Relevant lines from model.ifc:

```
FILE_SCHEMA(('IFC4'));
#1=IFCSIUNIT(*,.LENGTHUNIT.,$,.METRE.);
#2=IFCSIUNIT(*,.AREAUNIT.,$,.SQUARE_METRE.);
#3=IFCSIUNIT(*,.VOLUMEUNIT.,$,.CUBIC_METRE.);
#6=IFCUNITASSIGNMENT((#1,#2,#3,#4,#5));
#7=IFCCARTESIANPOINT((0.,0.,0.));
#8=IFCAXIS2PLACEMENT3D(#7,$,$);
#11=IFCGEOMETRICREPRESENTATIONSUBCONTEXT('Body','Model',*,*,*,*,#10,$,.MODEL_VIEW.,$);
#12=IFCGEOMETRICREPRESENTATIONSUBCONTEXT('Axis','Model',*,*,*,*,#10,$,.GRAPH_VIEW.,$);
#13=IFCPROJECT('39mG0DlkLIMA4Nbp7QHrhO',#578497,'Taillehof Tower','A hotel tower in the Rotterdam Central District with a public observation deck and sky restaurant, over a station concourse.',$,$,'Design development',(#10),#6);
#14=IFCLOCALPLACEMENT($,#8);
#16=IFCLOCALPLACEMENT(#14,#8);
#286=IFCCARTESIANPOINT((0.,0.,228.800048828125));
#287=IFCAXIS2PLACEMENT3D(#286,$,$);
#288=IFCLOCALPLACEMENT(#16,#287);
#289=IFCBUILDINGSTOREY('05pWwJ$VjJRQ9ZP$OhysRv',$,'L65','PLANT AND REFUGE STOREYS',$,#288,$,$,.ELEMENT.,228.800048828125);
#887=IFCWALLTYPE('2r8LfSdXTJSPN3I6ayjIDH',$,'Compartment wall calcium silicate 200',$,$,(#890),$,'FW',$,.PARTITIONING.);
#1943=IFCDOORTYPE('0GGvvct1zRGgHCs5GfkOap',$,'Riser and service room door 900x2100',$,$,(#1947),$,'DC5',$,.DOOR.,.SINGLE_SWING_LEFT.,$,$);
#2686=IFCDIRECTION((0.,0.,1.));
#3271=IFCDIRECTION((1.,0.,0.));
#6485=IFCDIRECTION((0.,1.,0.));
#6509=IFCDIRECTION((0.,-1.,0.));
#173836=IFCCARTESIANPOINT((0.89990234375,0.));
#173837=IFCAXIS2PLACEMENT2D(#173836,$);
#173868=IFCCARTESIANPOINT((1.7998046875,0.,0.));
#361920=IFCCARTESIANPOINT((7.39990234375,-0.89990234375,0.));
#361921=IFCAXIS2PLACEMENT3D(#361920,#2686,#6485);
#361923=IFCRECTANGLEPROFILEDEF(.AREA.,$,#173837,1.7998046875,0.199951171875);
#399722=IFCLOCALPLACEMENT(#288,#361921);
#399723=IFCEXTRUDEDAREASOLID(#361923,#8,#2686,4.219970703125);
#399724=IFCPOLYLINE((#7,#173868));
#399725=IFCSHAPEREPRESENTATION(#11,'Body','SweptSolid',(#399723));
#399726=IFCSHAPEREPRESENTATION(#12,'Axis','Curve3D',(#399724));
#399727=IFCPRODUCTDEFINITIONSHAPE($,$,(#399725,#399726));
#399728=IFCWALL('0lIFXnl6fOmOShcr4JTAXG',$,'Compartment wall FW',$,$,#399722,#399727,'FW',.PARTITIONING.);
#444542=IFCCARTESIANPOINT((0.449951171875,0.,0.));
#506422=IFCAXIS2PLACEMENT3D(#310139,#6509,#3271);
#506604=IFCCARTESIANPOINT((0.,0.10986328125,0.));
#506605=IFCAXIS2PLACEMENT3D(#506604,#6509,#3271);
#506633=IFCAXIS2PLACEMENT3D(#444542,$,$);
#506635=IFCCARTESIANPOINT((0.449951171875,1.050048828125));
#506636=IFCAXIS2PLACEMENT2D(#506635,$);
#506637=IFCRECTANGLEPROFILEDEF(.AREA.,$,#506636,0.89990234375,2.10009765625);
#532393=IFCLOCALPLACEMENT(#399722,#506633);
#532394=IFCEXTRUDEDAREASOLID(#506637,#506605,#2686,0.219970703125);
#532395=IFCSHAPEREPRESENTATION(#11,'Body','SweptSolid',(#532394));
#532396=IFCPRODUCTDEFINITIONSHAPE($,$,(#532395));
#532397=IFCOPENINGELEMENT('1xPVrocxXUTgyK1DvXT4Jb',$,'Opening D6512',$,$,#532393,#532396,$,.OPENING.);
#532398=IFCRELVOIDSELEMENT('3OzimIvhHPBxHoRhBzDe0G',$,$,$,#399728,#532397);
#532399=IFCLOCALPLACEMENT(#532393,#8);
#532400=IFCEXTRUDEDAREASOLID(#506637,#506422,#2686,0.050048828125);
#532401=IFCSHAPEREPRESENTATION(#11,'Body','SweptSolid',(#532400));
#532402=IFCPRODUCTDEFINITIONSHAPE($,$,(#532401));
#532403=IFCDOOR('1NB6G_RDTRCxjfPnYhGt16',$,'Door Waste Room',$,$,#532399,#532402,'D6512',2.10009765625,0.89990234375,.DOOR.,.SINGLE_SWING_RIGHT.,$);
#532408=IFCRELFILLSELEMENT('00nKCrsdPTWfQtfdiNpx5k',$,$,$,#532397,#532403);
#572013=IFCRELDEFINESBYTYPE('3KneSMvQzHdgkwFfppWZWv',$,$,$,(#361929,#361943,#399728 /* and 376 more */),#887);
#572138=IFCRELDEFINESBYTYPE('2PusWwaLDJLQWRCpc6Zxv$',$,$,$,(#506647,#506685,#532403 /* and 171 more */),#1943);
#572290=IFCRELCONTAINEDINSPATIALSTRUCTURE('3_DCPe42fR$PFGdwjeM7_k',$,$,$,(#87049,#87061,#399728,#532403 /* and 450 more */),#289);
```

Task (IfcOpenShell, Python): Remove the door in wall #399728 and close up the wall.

```python
import ifcopenshell
import ifcopenshell.api.feature
import ifcopenshell.api.root
import ifcopenshell.geom
import ifcopenshell.util.shape

model = ifcopenshell.open("model.ifc")
settings = ifcopenshell.geom.settings()


def volume(element):
    """Net volume in cubic metres, openings subtracted."""
    shape = ifcopenshell.geom.create_shape(settings, element)
    return ifcopenshell.util.shape.get_volume(shape.geometry)


door = model.by_guid("1NB6G_RDTRCxjfPnYhGt16")
opening = door.FillsVoids[0].RelatingOpeningElement
wall = opening.VoidsElements[0].RelatingBuildingElement
before = volume(wall)

ifcopenshell.api.root.remove_product(model, product=door)
ifcopenshell.api.feature.remove_feature(model, feature=opening)

after = volume(wall)

print(f"wall volume {before:.3f} -> {after:.3f} m3")

model.write("model_rev.ifc")
```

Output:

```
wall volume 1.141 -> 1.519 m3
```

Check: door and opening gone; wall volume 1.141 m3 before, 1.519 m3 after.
